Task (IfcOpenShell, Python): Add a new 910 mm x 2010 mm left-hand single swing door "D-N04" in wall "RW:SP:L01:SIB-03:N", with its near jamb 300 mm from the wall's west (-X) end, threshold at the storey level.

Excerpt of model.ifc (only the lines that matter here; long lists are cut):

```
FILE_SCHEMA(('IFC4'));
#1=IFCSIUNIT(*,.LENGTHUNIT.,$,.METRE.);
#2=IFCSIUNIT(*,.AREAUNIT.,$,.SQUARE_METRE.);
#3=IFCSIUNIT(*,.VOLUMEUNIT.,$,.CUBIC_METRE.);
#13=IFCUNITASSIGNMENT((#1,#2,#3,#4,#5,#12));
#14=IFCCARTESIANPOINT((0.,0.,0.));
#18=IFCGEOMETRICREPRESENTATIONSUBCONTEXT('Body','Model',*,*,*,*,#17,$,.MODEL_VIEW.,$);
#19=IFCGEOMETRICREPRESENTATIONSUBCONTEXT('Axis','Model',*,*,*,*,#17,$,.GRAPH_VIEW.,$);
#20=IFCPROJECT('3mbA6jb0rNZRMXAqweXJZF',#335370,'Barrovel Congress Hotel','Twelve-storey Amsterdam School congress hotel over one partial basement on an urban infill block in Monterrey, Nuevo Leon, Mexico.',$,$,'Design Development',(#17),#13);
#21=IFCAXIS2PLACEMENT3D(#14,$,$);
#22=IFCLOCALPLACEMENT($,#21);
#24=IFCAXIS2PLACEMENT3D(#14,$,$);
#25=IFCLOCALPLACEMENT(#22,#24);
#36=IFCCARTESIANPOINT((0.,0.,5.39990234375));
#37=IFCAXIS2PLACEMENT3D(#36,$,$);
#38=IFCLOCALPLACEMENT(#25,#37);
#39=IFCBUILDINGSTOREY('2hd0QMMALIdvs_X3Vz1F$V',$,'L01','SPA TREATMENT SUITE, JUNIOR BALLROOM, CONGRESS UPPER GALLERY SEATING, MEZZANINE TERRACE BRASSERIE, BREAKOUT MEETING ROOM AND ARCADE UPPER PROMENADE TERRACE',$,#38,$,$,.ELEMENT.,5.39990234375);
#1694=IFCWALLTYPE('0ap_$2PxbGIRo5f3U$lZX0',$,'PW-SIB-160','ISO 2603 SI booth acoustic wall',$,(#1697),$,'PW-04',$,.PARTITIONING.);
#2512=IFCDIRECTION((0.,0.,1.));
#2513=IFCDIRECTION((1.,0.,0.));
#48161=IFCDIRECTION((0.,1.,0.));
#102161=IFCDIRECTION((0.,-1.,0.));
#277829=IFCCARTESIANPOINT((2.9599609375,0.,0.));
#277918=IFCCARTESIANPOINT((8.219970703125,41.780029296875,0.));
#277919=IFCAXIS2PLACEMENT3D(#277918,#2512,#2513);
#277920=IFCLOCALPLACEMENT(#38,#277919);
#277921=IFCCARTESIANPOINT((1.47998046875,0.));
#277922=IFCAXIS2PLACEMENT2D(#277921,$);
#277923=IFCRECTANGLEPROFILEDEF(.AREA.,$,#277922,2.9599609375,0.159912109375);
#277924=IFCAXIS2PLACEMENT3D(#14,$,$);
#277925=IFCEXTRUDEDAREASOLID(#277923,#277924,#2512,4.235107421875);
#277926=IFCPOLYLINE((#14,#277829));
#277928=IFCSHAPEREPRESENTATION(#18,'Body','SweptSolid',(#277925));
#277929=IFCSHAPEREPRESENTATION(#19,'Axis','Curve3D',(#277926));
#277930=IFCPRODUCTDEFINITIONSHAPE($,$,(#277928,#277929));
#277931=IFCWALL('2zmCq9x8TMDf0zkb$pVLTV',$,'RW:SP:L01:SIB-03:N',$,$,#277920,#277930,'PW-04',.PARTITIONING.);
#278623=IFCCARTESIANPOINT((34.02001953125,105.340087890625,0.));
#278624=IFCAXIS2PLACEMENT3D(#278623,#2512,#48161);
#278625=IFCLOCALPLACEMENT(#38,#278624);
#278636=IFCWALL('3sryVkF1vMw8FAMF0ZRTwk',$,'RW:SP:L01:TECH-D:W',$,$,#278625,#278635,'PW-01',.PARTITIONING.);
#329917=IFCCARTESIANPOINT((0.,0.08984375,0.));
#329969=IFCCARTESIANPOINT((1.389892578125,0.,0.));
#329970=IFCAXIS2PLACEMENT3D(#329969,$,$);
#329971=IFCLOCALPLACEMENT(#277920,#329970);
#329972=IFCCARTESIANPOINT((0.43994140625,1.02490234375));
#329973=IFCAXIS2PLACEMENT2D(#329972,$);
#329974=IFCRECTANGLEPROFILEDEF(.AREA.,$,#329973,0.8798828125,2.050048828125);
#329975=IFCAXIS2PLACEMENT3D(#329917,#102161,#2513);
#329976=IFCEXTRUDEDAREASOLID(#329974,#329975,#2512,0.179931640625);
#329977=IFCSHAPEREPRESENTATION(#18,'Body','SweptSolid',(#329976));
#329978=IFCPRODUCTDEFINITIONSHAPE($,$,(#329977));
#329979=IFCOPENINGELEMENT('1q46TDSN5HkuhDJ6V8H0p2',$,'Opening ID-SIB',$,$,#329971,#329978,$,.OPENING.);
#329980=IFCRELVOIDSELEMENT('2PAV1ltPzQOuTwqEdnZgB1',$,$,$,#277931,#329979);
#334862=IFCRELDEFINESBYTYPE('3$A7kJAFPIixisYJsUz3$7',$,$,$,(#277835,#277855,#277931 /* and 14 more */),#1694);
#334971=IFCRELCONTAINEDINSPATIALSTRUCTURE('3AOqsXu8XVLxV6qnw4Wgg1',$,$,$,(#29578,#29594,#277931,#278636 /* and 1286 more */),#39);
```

```python
import numpy as np
import ifcopenshell
import ifcopenshell.api.feature
import ifcopenshell.api.geometry
import ifcopenshell.api.root
import ifcopenshell.api.spatial
import ifcopenshell.geom
import ifcopenshell.util.element
import ifcopenshell.util.placement
import ifcopenshell.util.representation
import ifcopenshell.util.shape
import ifcopenshell.util.unit

model = ifcopenshell.open("model.ifc")
unit_scale = ifcopenshell.util.unit.calculate_unit_scale(model)
settings = ifcopenshell.geom.settings()


def volume(element):
    """Net volume in cubic metres, openings subtracted."""
    shape = ifcopenshell.geom.create_shape(settings, element)
    return ifcopenshell.util.shape.get_volume(shape.geometry)


wall = model.by_guid("2zmCq9x8TMDf0zkb$pVLTV")
storey = ifcopenshell.util.element.get_container(wall, ifc_class="IfcBuildingStorey")
context = ifcopenshell.util.representation.get_context(model, "Model", "Body", "MODEL_VIEW")
before = volume(wall)

width, height, from_end, sill = 0.91, 2.01, 0.3, 0.0  # metres

# The wall runs along its own X axis, and the end named is its -X end.
wall_shape = ifcopenshell.geom.create_shape(settings, wall)
x, y, z = ifcopenshell.util.shape.get_vertices(wall_shape.geometry).T
start = x.min() + from_end
face, thickness = float(y.min()), float(y.max() - y.min())
wall_matrix = ifcopenshell.util.placement.get_local_placement(wall.ObjectPlacement)
level = ifcopenshell.util.placement.get_local_placement(storey.ObjectPlacement)[2, 3]


def in_wall(x, y):
    """Placement at x, y metres in the wall's axes, at sill height."""
    matrix = wall_matrix.copy()
    matrix[:, 3] = wall_matrix @ np.array([x / unit_scale, y / unit_scale, 0.0, 1.0])
    matrix[2, 3] = level + sill / unit_scale
    return matrix


# Opening: a box that overshoots both wall faces by 50 mm.
opening = ifcopenshell.api.root.create_entity(model, ifc_class="IfcOpeningElement", predefined_type="OPENING")
box = ifcopenshell.api.geometry.add_wall_representation(
    model, context=context, length=width, height=height, thickness=thickness + 0.1
)
ifcopenshell.api.geometry.assign_representation(model, product=opening, representation=box)
ifcopenshell.api.geometry.edit_object_placement(model, product=opening, matrix=in_wall(start, face - 0.05), is_si=False)
ifcopenshell.api.feature.add_feature(model, feature=opening, element=wall)

door = ifcopenshell.api.root.create_entity(model, ifc_class="IfcDoor", name="D-N04", predefined_type="DOOR")
door.OverallWidth, door.OverallHeight = width / unit_scale, height / unit_scale
door.OperationType = "SINGLE_SWING_LEFT"
body = ifcopenshell.api.geometry.add_door_representation(
    model,
    context=context,
    overall_width=door.OverallWidth,
    overall_height=door.OverallHeight,
    operation_type="SINGLE_SWING_LEFT",
    lining_properties={"LiningDepth": thickness / unit_scale, "ThresholdDepth": thickness / unit_scale},
)
ifcopenshell.api.geometry.assign_representation(model, product=door, representation=body)
ifcopenshell.api.spatial.assign_container(model, products=[door], relating_structure=storey)
ifcopenshell.api.feature.add_filling(model, opening=opening, element=door)

# The lining spans the wall, so the door starts at the wall face.
ifcopenshell.api.geometry.edit_object_placement(model, product=door, matrix=in_wall(start, face), is_si=False)

after = volume(wall)

print(f"wall volume {before:.3f} -> {after:.3f} m3")

model.write("model_rev.ifc")
```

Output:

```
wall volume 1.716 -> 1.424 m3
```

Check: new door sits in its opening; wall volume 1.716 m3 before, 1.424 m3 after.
